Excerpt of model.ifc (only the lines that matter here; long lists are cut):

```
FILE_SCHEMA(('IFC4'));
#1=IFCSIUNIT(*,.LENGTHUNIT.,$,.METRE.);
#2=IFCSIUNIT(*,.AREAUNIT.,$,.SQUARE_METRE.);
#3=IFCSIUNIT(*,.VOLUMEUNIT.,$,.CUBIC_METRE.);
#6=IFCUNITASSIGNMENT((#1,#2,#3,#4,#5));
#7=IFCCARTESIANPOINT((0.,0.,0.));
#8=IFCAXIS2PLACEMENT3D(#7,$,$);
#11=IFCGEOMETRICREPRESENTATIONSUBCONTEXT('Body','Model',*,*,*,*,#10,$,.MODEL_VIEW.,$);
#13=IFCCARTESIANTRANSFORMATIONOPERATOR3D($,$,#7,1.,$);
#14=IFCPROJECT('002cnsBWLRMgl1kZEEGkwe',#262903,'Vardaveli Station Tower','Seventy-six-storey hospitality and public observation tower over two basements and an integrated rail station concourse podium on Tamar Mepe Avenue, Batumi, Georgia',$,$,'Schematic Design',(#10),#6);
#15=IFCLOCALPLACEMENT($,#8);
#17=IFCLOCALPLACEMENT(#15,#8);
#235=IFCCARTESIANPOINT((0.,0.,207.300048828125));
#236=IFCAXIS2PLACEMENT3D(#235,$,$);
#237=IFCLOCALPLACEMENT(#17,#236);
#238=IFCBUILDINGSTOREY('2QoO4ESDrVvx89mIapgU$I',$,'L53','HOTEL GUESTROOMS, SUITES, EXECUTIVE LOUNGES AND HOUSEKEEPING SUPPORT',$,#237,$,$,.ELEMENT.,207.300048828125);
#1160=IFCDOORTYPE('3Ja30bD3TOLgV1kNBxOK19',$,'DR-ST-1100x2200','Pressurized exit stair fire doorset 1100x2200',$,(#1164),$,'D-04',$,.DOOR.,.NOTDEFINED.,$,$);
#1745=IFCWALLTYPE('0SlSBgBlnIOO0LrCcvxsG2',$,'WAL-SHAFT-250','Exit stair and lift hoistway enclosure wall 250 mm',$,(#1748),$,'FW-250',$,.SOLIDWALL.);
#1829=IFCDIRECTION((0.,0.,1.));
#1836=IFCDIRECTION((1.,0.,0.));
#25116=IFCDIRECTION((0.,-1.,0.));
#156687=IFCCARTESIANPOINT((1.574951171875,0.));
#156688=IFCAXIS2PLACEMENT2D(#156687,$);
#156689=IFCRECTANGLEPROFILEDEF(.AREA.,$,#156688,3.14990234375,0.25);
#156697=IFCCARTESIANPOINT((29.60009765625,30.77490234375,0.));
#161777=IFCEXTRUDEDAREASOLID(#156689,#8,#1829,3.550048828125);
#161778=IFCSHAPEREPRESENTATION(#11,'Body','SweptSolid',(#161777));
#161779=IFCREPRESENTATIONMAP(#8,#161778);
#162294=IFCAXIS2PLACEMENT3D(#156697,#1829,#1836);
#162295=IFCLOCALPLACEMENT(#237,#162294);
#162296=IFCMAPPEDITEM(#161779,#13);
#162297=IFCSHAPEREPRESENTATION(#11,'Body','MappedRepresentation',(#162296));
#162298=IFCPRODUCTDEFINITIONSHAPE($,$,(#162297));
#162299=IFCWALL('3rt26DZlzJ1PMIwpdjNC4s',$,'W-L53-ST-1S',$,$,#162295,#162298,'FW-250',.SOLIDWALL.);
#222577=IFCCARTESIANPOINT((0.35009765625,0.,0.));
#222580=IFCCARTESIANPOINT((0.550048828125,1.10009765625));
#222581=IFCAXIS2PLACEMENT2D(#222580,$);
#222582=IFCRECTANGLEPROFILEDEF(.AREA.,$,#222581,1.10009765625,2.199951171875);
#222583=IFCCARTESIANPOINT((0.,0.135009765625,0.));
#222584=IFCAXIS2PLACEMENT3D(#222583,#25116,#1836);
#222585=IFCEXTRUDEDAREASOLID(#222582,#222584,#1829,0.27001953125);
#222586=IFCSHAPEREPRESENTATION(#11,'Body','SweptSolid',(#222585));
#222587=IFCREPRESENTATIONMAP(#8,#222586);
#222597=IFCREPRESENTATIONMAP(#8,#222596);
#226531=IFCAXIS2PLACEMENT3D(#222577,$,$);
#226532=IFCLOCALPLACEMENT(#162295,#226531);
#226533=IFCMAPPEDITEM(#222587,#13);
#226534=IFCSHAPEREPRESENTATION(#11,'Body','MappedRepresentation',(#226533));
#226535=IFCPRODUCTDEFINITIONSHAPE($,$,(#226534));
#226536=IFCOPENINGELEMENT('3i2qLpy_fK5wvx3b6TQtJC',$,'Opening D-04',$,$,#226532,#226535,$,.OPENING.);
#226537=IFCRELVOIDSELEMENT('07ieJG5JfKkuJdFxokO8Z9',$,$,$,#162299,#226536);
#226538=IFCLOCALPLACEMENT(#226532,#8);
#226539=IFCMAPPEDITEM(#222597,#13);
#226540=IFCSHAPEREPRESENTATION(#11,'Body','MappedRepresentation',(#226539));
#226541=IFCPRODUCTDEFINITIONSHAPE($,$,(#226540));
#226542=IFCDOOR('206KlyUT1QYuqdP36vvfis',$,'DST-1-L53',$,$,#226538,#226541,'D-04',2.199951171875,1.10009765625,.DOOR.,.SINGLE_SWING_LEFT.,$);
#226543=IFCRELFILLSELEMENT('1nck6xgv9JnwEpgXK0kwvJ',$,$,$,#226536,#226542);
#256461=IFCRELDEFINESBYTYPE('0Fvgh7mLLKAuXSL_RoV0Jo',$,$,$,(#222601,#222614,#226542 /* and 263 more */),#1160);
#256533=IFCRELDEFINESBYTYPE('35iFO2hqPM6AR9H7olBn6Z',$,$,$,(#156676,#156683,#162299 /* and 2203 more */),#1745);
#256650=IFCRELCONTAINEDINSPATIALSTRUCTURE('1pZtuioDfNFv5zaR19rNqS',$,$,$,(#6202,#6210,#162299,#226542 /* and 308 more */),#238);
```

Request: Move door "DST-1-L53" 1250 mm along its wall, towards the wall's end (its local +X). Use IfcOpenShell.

```python
import ifcopenshell
import ifcopenshell.api.geometry
import ifcopenshell.util.placement

model = ifcopenshell.open("model.ifc")

door = model.by_guid("206KlyUT1QYuqdP36vvfis")
opening = door.FillsVoids[0].RelatingOpeningElement
wall = opening.VoidsElements[0].RelatingBuildingElement

wall_matrix = ifcopenshell.util.placement.get_local_placement(wall.ObjectPlacement)
shift = wall_matrix[:3, 0] * 1.25
before = ifcopenshell.util.placement.get_local_placement(door.ObjectPlacement)[:3, 3].copy()

# The door is placed relative to its opening, so it follows when the opening moves.
matrix = ifcopenshell.util.placement.get_local_placement(opening.ObjectPlacement)
matrix[:3, 3] += shift
ifcopenshell.api.geometry.edit_object_placement(
    model, product=opening, matrix=matrix, is_si=False, should_transform_children=True
)

after = ifcopenshell.util.placement.get_local_placement(door.ObjectPlacement)[:3, 3]
print("door moved by", (after - before).round(3) + 0.0)

model.write("model_v2.ifc")
```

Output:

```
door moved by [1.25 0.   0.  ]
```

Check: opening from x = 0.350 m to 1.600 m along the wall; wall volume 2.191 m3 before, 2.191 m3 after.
